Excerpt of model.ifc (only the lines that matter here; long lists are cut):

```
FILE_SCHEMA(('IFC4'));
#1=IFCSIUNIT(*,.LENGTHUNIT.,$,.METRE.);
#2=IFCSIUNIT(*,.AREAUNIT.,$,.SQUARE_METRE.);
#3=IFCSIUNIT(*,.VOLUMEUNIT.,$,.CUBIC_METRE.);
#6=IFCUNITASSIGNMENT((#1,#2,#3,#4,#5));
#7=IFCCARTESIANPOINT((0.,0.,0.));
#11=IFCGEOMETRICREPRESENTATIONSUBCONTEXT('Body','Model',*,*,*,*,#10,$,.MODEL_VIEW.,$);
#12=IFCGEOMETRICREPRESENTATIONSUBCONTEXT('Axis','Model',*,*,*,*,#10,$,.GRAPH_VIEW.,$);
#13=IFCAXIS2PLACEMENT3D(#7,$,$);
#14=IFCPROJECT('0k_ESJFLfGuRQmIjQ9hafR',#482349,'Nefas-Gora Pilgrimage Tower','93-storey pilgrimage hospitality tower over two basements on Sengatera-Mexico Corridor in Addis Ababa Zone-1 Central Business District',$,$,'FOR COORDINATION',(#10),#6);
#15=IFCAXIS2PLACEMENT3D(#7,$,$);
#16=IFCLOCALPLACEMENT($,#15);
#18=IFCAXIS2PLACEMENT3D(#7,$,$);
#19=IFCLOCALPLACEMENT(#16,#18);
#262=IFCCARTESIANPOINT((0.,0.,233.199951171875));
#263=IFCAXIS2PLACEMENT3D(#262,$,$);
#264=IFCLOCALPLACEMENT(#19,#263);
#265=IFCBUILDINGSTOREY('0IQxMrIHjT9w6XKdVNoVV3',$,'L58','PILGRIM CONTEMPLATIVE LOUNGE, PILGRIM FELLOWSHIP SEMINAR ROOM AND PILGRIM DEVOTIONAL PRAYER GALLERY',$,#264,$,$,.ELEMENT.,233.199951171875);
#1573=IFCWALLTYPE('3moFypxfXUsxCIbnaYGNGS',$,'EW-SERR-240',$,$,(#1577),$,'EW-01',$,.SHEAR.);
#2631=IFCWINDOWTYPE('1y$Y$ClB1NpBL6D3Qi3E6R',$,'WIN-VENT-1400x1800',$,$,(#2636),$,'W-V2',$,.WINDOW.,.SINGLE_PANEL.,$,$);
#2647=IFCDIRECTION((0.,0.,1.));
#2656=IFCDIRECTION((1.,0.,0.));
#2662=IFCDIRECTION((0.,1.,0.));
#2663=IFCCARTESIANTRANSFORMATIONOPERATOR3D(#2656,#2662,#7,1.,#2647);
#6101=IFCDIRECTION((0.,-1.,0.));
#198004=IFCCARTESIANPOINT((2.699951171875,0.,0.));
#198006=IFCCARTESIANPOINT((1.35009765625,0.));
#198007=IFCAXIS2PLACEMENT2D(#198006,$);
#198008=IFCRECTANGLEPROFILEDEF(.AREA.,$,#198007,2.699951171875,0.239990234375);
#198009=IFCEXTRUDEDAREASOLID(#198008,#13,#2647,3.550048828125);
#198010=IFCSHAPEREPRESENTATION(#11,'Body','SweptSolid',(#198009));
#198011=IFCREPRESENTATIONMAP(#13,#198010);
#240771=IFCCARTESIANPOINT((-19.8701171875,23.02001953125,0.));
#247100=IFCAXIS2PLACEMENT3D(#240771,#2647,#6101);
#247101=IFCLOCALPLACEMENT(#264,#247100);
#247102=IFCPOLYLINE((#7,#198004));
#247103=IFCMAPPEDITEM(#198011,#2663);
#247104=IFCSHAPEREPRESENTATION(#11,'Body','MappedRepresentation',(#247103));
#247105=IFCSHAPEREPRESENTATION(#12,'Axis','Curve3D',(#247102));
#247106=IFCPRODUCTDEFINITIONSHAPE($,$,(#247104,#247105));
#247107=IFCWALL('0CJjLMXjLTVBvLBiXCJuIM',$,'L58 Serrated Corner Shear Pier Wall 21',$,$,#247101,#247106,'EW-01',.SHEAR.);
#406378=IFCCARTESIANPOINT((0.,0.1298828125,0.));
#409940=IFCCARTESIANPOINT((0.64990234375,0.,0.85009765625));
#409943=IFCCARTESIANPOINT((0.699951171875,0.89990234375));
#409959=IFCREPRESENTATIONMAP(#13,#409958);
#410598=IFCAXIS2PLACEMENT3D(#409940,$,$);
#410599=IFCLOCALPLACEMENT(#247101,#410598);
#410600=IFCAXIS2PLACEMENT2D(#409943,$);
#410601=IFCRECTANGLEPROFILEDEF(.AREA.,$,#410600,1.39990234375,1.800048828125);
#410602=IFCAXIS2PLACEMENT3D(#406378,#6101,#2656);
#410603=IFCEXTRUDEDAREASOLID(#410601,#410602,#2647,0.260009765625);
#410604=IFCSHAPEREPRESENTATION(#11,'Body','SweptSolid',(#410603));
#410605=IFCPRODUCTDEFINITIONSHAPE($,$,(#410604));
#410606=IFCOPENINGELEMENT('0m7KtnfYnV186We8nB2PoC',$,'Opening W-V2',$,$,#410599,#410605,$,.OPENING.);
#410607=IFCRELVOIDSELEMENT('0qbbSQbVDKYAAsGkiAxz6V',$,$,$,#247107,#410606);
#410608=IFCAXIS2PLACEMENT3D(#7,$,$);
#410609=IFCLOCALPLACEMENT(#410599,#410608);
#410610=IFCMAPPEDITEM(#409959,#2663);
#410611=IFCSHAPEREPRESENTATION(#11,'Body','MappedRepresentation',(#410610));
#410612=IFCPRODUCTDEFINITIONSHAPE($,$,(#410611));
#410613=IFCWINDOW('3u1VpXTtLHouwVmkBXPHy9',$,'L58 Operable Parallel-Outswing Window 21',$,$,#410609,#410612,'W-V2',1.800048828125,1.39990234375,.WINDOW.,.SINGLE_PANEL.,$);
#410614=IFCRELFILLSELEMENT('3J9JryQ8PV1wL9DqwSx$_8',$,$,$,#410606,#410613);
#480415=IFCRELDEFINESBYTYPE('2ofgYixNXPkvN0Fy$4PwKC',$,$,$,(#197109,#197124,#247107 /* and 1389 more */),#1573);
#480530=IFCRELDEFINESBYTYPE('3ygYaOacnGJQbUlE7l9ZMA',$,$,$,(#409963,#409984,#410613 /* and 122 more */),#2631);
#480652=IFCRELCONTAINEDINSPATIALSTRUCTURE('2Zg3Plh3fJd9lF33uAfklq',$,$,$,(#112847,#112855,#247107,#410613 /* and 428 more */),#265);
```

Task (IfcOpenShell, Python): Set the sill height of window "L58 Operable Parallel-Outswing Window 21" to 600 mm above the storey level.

```python
import numpy as np
import ifcopenshell
import ifcopenshell.api.geometry
import ifcopenshell.geom
import ifcopenshell.util.element
import ifcopenshell.util.placement
import ifcopenshell.util.shape
import ifcopenshell.util.unit

model = ifcopenshell.open("model.ifc")
unit_scale = ifcopenshell.util.unit.calculate_unit_scale(model)

window = model.by_guid("3u1VpXTtLHouwVmkBXPHy9")
opening = window.FillsVoids[0].RelatingOpeningElement
storey = ifcopenshell.util.element.get_container(window, ifc_class="IfcBuildingStorey")
level = ifcopenshell.util.placement.get_local_placement(storey.ObjectPlacement)[2, 3]

# The opening's origin need not be at the sill, so measure its lowest point.
shape = ifcopenshell.geom.create_shape(ifcopenshell.geom.settings(), opening)
bottom = ifcopenshell.util.shape.get_shape_bottom_elevation(shape, shape.geometry) / unit_scale
dz = level + 0.6 / unit_scale - bottom

shift = np.array([0.0, 0.0, dz])
# The window is placed relative to its opening, so it follows when the opening moves.
matrix = ifcopenshell.util.placement.get_local_placement(opening.ObjectPlacement)
matrix[:3, 3] += shift
ifcopenshell.api.geometry.edit_object_placement(
    model, product=opening, matrix=matrix, is_si=False, should_transform_children=True
)

print(f"moved by {dz * unit_scale:+.3f} m")

model.write("model-out.ifc")
```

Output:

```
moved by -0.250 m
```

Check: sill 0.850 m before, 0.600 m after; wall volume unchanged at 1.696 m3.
